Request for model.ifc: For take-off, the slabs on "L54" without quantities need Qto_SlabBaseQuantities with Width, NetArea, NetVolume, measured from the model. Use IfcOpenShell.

First a look at what the model holds.

```python
import ifcopenshell
import ifcopenshell.util.element
import ifcopenshell.util.unit

model = ifcopenshell.open("model.ifc")
print(model.schema)
for unit_type in ("LENGTHUNIT", "AREAUNIT", "VOLUMEUNIT"):
    print(unit_type, ifcopenshell.util.unit.calculate_unit_scale(model, unit_type))
storey = next(s for s in model.by_type("IfcBuildingStorey") if s.Name == "L54")
slabs = [e for e in ifcopenshell.util.element.get_decomposition(storey) if e.is_a("IfcSlab")]
for e in sorted(slabs, key=lambda e: e.id()):
    print(e.id(), e.is_a(), e.Name, list(ifcopenshell.util.element.get_psets(e, qtos_only=True)), sep=" | ")
```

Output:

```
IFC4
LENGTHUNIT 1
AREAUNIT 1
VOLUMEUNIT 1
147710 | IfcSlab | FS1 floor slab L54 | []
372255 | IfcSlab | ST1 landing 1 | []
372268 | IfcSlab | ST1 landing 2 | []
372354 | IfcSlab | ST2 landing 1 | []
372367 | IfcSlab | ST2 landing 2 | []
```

```python
import ifcopenshell
import ifcopenshell.api.pset
import ifcopenshell.geom
import ifcopenshell.util.element
import ifcopenshell.util.shape
import ifcopenshell.util.unit

model = ifcopenshell.open("model.ifc")
unit_scale = ifcopenshell.util.unit.calculate_unit_scale(model)
area_scale = ifcopenshell.util.unit.calculate_unit_scale(model, "AREAUNIT")
volume_scale = ifcopenshell.util.unit.calculate_unit_scale(model, "VOLUMEUNIT")
settings = ifcopenshell.geom.settings()

storey = next(s for s in model.by_type("IfcBuildingStorey") if s.Name == "L54")
slabs = [e for e in ifcopenshell.util.element.get_decomposition(storey) if e.is_a("IfcSlab")]

for e in sorted(slabs, key=lambda e: e.id()):
    if ifcopenshell.util.element.get_psets(e, qtos_only=True, should_inherit=False):
        continue
    # Geometry comes back in metres, in the element's own axes.
    shape = ifcopenshell.geom.create_shape(settings, e)
    values = {
        "Width": ifcopenshell.util.shape.get_z(shape.geometry) / unit_scale,
        "NetArea": ifcopenshell.util.shape.get_footprint_area(shape.geometry) / area_scale,
        "NetVolume": ifcopenshell.util.shape.get_volume(shape.geometry) / volume_scale,
    }
    qto = ifcopenshell.api.pset.add_qto(model, product=e, name="Qto_SlabBaseQuantities")
    ifcopenshell.api.pset.edit_qto(model, qto=qto, properties=values)
    print(e.id(), {k: round(v, 3) for k, v in values.items()})

model.write("model_v2.ifc")
```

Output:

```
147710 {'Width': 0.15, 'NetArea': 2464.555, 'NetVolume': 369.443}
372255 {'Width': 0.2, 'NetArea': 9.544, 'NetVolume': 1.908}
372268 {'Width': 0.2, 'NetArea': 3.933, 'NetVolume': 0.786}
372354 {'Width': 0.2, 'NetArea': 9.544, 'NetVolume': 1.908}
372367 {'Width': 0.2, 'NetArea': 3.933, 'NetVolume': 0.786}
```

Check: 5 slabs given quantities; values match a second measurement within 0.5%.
